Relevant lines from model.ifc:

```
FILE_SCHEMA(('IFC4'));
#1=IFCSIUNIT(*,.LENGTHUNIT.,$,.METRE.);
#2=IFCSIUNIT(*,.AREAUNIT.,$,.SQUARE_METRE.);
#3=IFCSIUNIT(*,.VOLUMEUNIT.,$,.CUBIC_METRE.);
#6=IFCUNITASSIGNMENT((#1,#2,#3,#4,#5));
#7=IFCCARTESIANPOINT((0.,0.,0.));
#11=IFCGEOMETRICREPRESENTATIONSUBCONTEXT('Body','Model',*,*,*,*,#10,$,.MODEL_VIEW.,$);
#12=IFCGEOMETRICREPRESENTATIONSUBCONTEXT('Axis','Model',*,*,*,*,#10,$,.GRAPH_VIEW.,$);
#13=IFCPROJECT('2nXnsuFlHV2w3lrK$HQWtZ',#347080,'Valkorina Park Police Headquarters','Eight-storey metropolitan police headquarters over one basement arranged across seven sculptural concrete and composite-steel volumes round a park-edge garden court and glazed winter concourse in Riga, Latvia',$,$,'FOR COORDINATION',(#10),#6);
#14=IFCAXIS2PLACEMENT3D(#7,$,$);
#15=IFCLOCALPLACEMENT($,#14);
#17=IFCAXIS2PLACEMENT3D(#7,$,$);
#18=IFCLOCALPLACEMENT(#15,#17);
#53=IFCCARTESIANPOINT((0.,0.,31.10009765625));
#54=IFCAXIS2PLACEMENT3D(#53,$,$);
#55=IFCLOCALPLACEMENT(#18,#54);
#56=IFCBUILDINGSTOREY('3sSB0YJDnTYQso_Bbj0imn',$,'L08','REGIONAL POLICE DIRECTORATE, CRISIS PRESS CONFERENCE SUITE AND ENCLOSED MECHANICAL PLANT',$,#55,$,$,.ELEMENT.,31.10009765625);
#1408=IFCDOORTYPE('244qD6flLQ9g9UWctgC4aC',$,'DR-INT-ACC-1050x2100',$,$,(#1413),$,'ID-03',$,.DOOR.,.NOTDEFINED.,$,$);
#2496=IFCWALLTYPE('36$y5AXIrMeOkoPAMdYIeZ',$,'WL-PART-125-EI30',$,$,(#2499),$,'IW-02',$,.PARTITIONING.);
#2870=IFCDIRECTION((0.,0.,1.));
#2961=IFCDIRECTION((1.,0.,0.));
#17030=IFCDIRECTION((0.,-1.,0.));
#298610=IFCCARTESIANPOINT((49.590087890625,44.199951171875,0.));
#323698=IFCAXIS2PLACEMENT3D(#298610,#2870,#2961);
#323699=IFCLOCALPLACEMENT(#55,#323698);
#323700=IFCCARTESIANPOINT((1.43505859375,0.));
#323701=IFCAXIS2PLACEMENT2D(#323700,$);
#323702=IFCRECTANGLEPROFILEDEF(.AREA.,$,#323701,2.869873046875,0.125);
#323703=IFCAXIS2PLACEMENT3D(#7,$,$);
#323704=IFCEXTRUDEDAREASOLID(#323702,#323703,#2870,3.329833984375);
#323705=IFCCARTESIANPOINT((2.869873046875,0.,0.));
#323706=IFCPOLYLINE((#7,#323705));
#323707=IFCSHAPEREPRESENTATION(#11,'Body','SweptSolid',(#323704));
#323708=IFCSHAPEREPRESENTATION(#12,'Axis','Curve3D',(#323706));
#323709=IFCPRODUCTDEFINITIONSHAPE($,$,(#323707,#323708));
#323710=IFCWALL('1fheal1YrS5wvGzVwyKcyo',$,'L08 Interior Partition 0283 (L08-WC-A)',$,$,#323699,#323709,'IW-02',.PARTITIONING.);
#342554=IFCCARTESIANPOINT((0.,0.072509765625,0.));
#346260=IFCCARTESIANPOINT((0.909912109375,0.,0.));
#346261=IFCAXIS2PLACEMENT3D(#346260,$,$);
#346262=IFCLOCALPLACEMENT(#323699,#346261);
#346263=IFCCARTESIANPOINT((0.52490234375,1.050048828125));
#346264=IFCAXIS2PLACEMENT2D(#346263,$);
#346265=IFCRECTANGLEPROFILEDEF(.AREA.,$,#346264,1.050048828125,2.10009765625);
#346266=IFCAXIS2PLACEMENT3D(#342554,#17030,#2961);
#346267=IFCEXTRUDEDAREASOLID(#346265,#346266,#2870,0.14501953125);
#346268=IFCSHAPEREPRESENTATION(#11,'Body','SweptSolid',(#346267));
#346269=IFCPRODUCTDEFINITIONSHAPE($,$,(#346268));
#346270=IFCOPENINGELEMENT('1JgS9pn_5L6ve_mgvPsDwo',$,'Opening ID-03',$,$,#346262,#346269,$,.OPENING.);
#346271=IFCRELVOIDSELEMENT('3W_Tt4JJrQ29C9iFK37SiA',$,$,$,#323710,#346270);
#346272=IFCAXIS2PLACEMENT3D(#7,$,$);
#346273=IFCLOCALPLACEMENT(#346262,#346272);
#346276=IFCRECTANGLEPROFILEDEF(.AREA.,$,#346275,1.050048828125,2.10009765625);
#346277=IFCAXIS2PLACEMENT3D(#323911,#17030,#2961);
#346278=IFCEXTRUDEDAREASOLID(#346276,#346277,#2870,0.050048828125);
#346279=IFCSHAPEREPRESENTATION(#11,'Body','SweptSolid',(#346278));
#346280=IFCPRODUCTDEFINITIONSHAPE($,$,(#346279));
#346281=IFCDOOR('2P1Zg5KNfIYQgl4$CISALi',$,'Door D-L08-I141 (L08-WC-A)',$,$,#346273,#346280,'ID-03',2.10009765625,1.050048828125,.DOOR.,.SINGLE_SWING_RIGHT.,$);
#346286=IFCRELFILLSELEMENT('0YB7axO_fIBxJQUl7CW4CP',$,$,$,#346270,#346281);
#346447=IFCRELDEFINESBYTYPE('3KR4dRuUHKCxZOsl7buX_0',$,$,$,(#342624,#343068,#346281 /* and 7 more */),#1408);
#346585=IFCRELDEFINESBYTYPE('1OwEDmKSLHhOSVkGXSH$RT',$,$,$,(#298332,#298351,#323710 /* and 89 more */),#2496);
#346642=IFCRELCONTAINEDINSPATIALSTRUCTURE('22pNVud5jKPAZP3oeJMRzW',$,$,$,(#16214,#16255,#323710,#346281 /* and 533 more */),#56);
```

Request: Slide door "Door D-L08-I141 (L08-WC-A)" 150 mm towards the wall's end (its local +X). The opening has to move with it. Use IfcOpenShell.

```python
import ifcopenshell
import ifcopenshell.api.geometry
import ifcopenshell.util.placement

model = ifcopenshell.open("model.ifc")

door = model.by_guid("2P1Zg5KNfIYQgl4$CISALi")
opening = door.FillsVoids[0].RelatingOpeningElement
wall = opening.VoidsElements[0].RelatingBuildingElement

wall_matrix = ifcopenshell.util.placement.get_local_placement(wall.ObjectPlacement)
shift = wall_matrix[:3, 0] * 0.15
before = ifcopenshell.util.placement.get_local_placement(door.ObjectPlacement)[:3, 3].copy()

# The door is placed relative to its opening, so it follows when the opening moves.
matrix = ifcopenshell.util.placement.get_local_placement(opening.ObjectPlacement)
matrix[:3, 3] += shift
ifcopenshell.api.geometry.edit_object_placement(
    model, product=opening, matrix=matrix, is_si=False, should_transform_children=True
)

after = ifcopenshell.util.placement.get_local_placement(door.ObjectPlacement)[:3, 3]
print("door moved by", (after - before).round(3) + 0.0)

model.write("model-out.ifc")
```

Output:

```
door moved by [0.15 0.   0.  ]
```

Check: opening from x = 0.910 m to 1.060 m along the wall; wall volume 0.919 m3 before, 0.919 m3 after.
